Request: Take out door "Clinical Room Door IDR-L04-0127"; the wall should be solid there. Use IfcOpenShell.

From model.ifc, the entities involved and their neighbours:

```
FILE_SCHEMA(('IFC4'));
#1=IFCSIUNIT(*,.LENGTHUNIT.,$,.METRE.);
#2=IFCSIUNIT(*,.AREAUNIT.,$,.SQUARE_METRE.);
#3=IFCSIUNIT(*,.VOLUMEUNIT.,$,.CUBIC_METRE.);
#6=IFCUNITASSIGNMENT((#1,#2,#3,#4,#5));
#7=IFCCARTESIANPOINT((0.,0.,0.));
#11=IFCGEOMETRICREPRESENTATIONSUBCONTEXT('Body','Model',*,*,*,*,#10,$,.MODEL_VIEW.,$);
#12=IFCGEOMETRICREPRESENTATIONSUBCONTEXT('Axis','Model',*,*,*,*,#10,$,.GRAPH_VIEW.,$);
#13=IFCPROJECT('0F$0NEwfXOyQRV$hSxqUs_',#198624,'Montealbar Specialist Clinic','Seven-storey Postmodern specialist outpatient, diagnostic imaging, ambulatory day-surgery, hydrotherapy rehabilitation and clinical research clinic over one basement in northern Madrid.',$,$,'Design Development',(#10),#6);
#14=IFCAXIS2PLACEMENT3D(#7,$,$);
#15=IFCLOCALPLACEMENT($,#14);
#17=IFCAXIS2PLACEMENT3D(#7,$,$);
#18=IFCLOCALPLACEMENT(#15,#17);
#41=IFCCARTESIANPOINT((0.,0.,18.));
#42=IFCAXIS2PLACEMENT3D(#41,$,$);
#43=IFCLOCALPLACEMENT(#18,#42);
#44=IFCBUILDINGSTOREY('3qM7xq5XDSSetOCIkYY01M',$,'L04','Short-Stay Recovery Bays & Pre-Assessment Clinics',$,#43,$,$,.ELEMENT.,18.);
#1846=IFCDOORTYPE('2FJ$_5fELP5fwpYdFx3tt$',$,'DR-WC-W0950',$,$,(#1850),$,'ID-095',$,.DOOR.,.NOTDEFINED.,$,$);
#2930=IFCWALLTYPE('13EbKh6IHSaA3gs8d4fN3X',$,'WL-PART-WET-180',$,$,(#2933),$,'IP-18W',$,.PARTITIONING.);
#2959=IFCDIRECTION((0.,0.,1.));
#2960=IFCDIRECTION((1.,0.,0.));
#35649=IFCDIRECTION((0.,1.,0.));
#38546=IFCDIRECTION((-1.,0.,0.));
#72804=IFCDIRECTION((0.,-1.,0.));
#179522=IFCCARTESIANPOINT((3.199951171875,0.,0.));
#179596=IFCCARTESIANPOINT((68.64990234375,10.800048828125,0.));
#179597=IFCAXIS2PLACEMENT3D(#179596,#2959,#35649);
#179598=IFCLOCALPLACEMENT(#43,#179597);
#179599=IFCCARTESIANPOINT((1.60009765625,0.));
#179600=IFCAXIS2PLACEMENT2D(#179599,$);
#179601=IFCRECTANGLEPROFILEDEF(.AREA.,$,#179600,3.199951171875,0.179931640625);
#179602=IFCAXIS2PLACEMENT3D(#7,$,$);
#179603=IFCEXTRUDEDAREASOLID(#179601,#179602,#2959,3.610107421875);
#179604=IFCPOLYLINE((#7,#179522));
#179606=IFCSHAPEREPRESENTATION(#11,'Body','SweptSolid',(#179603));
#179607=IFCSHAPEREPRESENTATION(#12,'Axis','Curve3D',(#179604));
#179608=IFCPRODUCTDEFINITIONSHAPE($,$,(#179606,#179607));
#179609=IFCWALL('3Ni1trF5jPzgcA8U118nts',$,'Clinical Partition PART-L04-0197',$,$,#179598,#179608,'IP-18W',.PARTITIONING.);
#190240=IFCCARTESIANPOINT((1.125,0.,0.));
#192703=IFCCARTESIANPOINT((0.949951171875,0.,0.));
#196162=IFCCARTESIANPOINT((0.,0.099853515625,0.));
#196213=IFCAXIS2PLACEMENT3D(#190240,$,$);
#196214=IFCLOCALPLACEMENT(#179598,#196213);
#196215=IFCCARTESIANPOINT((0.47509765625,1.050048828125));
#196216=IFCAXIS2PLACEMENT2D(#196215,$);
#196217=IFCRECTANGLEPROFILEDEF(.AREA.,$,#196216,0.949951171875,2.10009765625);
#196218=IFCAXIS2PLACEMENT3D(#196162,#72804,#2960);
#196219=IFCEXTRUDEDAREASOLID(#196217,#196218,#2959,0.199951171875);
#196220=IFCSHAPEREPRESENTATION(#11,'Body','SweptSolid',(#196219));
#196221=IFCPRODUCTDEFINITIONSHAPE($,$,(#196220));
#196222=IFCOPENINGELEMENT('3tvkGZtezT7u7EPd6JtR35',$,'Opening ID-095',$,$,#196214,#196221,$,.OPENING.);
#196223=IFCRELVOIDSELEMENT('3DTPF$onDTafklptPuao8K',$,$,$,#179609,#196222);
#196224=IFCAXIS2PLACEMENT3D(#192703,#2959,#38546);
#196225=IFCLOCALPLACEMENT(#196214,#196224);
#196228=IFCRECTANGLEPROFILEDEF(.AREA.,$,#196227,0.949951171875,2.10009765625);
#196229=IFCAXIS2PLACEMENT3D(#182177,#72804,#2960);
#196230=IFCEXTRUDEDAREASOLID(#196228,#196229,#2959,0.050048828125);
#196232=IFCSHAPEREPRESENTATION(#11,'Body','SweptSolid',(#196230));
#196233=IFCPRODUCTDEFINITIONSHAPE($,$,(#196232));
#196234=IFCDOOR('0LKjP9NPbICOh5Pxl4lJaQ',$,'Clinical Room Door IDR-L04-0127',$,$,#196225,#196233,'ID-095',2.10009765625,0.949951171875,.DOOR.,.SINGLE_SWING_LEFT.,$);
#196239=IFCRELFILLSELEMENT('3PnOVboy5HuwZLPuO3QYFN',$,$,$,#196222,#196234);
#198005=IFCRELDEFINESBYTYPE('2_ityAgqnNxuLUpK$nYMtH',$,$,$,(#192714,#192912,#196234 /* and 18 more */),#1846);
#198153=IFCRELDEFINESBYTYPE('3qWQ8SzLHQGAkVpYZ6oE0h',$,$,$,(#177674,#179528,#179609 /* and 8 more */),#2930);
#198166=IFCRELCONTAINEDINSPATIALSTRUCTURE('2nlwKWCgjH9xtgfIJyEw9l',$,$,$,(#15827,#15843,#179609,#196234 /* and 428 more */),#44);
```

```python
import ifcopenshell
import ifcopenshell.api.feature
import ifcopenshell.api.root
import ifcopenshell.geom
import ifcopenshell.util.shape

model = ifcopenshell.open("model.ifc")
settings = ifcopenshell.geom.settings()


def volume(element):
    """Net volume in cubic metres, openings subtracted."""
    shape = ifcopenshell.geom.create_shape(settings, element)
    return ifcopenshell.util.shape.get_volume(shape.geometry)


door = model.by_guid("0LKjP9NPbICOh5Pxl4lJaQ")
opening = door.FillsVoids[0].RelatingOpeningElement
wall = opening.VoidsElements[0].RelatingBuildingElement
before = volume(wall)

ifcopenshell.api.root.remove_product(model, product=door)
ifcopenshell.api.feature.remove_feature(model, feature=opening)

after = volume(wall)

print(f"wall volume {before:.3f} -> {after:.3f} m3")

model.write("model_edited.ifc")
```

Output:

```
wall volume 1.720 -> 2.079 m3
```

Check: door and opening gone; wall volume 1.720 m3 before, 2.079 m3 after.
